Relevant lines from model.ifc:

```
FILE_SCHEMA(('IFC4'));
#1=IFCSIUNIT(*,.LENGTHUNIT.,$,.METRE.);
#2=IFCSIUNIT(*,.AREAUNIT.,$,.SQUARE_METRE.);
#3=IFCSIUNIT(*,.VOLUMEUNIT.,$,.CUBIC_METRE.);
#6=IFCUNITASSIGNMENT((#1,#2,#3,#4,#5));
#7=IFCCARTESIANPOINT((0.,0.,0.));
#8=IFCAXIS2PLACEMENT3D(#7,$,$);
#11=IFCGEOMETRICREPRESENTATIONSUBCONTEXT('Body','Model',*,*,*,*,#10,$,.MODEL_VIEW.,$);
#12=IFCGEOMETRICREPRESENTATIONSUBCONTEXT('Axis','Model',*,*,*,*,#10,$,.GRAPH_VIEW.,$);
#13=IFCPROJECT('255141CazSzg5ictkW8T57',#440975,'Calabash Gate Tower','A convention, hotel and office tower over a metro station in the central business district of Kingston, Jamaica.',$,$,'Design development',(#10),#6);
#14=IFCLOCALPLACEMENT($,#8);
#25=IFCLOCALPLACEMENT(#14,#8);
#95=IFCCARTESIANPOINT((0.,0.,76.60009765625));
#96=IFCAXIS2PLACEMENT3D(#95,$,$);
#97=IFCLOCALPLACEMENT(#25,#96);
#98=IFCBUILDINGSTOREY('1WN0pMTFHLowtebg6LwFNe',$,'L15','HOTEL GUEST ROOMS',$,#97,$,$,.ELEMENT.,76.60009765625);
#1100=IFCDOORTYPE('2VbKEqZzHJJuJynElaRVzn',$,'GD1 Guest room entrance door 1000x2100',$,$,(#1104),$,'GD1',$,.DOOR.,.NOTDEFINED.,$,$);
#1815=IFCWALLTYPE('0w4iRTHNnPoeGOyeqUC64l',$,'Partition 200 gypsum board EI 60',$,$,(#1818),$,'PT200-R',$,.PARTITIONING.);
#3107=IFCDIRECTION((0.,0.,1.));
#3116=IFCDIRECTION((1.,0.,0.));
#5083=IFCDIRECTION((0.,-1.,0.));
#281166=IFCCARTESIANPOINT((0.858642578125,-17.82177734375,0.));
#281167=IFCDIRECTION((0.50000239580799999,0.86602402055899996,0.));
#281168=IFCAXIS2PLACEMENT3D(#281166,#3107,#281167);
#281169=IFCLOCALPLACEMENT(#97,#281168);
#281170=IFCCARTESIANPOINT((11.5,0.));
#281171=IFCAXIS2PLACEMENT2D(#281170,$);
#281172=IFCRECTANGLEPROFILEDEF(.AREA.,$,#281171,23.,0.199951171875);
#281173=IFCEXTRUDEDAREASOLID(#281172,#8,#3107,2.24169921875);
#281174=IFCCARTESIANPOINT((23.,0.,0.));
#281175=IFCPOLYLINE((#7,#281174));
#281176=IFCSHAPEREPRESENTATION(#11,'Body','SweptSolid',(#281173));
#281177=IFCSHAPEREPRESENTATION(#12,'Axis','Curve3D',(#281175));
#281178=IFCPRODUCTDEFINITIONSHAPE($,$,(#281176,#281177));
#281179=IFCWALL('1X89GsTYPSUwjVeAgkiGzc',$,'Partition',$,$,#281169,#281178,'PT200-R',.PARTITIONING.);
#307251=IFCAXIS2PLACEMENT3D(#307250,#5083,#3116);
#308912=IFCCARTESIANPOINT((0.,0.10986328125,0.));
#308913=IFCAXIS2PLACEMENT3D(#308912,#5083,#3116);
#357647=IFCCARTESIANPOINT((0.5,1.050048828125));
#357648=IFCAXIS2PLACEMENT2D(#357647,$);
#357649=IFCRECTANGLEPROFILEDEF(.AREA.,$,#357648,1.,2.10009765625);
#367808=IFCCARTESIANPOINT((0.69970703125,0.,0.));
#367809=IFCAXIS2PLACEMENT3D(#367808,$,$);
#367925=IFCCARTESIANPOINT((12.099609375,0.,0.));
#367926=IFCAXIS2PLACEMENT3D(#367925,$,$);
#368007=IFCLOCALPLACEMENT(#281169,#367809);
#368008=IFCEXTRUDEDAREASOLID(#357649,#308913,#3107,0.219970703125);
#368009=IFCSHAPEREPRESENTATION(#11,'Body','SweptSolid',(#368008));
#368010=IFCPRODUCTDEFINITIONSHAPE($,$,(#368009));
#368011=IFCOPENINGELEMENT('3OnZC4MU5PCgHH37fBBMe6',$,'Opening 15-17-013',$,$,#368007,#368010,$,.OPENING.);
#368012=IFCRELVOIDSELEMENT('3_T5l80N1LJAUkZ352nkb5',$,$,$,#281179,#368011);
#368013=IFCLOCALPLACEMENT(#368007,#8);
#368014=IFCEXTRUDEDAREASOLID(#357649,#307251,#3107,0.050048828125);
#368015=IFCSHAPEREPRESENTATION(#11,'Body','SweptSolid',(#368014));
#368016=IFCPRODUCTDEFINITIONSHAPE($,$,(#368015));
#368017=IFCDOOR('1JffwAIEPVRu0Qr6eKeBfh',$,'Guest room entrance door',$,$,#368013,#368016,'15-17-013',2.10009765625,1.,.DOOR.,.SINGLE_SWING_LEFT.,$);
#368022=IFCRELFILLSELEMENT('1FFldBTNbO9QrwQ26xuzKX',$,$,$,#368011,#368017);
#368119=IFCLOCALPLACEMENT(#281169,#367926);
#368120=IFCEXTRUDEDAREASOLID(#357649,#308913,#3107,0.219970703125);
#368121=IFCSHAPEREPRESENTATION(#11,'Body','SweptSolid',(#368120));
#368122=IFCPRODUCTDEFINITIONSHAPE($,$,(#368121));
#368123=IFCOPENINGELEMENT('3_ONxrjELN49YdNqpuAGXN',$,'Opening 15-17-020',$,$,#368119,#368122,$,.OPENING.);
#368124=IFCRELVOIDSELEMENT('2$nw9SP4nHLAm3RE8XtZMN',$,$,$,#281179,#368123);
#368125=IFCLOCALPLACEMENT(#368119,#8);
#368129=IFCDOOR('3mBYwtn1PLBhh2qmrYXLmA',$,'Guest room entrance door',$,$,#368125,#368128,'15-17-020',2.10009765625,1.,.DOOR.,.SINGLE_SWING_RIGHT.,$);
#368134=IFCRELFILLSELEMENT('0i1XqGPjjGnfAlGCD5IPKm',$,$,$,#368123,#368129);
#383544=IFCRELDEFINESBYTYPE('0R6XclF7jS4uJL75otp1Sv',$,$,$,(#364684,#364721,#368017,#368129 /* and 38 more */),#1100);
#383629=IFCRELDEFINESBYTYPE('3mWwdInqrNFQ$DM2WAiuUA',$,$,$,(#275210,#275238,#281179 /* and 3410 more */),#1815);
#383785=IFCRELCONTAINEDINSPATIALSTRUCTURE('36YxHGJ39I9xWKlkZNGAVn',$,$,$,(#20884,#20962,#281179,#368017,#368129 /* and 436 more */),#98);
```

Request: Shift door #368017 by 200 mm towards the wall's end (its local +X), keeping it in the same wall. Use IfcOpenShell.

```python
import ifcopenshell
import ifcopenshell.api.geometry
import ifcopenshell.util.placement

model = ifcopenshell.open("model.ifc")

door = model.by_guid("1JffwAIEPVRu0Qr6eKeBfh")
opening = door.FillsVoids[0].RelatingOpeningElement
wall = opening.VoidsElements[0].RelatingBuildingElement

wall_matrix = ifcopenshell.util.placement.get_local_placement(wall.ObjectPlacement)
shift = wall_matrix[:3, 0] * 0.2
before = ifcopenshell.util.placement.get_local_placement(door.ObjectPlacement)[:3, 3].copy()

# The door is placed relative to its opening, so it follows when the opening moves.
matrix = ifcopenshell.util.placement.get_local_placement(opening.ObjectPlacement)
matrix[:3, 3] += shift
ifcopenshell.api.geometry.edit_object_placement(
    model, product=opening, matrix=matrix, is_si=False, should_transform_children=True
)

after = ifcopenshell.util.placement.get_local_placement(door.ObjectPlacement)[:3, 3]
print("door moved by", (after - before).round(3) + 0.0)

model.write("model_rev.ifc")
```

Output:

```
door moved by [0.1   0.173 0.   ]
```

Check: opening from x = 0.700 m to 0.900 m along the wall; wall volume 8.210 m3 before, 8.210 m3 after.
